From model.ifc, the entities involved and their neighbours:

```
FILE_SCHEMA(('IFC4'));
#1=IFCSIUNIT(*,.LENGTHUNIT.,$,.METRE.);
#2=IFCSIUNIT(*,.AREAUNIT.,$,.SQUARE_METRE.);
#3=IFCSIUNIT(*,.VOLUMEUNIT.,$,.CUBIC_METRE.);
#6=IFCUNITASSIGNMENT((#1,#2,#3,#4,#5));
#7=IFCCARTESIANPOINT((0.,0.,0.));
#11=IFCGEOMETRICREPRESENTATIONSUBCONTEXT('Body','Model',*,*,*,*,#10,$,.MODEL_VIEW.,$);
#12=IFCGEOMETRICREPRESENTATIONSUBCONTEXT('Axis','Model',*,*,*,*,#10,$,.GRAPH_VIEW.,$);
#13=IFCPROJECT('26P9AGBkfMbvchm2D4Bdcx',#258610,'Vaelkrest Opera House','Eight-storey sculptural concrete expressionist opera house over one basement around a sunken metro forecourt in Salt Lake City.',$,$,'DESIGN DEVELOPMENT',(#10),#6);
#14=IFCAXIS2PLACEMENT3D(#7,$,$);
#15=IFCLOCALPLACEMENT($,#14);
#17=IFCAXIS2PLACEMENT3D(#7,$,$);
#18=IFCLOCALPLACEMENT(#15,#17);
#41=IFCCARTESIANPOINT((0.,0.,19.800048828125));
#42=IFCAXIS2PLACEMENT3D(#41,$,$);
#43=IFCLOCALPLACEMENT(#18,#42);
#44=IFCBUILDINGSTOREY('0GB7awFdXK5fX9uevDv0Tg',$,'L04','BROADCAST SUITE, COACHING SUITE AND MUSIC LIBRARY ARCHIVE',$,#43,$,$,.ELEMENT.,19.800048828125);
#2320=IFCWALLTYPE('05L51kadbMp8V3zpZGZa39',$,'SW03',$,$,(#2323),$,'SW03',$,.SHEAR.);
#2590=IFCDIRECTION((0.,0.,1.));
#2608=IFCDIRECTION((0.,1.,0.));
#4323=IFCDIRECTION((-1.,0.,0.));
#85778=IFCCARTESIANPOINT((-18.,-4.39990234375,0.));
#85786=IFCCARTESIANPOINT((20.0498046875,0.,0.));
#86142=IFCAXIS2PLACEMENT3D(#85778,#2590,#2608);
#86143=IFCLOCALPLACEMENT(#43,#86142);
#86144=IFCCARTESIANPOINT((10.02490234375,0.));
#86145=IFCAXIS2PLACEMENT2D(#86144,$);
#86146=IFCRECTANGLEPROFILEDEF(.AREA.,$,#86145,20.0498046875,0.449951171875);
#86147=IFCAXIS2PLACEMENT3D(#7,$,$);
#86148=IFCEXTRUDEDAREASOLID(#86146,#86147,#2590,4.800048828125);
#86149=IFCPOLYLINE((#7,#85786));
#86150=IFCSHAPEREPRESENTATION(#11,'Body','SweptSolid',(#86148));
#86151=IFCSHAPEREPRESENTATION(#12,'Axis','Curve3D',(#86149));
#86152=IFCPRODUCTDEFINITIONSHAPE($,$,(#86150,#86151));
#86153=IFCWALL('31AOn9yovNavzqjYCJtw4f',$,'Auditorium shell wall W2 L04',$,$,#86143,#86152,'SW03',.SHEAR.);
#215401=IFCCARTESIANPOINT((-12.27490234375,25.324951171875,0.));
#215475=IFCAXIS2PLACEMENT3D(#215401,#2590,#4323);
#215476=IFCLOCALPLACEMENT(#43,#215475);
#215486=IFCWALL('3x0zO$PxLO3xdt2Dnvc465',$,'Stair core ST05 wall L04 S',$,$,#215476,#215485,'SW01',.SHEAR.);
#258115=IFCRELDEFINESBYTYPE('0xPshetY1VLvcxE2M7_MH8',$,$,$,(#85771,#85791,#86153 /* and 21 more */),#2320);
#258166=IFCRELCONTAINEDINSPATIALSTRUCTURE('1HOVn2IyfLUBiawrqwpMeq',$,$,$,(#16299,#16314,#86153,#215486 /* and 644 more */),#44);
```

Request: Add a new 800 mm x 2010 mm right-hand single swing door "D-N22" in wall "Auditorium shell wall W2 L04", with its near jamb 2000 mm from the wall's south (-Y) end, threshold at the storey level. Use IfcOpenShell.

```python
import numpy as np
import ifcopenshell
import ifcopenshell.api.feature
import ifcopenshell.api.geometry
import ifcopenshell.api.root
import ifcopenshell.api.spatial
import ifcopenshell.geom
import ifcopenshell.util.element
import ifcopenshell.util.placement
import ifcopenshell.util.representation
import ifcopenshell.util.shape
import ifcopenshell.util.unit

model = ifcopenshell.open("model.ifc")
unit_scale = ifcopenshell.util.unit.calculate_unit_scale(model)
settings = ifcopenshell.geom.settings()


def volume(element):
    """Net volume in cubic metres, openings subtracted."""
    shape = ifcopenshell.geom.create_shape(settings, element)
    return ifcopenshell.util.shape.get_volume(shape.geometry)


wall = model.by_guid("31AOn9yovNavzqjYCJtw4f")
storey = ifcopenshell.util.element.get_container(wall, ifc_class="IfcBuildingStorey")
context = ifcopenshell.util.representation.get_context(model, "Model", "Body", "MODEL_VIEW")
before = volume(wall)

width, height, from_end, sill = 0.8, 2.01, 2, 0.0  # metres

# The wall runs along its own X axis, and the end named is its -X end.
wall_shape = ifcopenshell.geom.create_shape(settings, wall)
x, y, z = ifcopenshell.util.shape.get_vertices(wall_shape.geometry).T
start = x.min() + from_end
face, thickness = float(y.min()), float(y.max() - y.min())
wall_matrix = ifcopenshell.util.placement.get_local_placement(wall.ObjectPlacement)
level = ifcopenshell.util.placement.get_local_placement(storey.ObjectPlacement)[2, 3]


def in_wall(x, y):
    """Placement at x, y metres in the wall's axes, at sill height."""
    matrix = wall_matrix.copy()
    matrix[:, 3] = wall_matrix @ np.array([x / unit_scale, y / unit_scale, 0.0, 1.0])
    matrix[2, 3] = level + sill / unit_scale
    return matrix


# Opening: a box that overshoots both wall faces by 50 mm.
opening = ifcopenshell.api.root.create_entity(model, ifc_class="IfcOpeningElement", predefined_type="OPENING")
box = ifcopenshell.api.geometry.add_wall_representation(
    model, context=context, length=width, height=height, thickness=thickness + 0.1
)
ifcopenshell.api.geometry.assign_representation(model, product=opening, representation=box)
ifcopenshell.api.geometry.edit_object_placement(model, product=opening, matrix=in_wall(start, face - 0.05), is_si=False)
ifcopenshell.api.feature.add_feature(model, feature=opening, element=wall)

door = ifcopenshell.api.root.create_entity(model, ifc_class="IfcDoor", name="D-N22", predefined_type="DOOR")
door.OverallWidth, door.OverallHeight = width / unit_scale, height / unit_scale
door.OperationType = "SINGLE_SWING_RIGHT"
body = ifcopenshell.api.geometry.add_door_representation(
    model,
    context=context,
    overall_width=door.OverallWidth,
    overall_height=door.OverallHeight,
    operation_type="SINGLE_SWING_RIGHT",
    lining_properties={"LiningDepth": thickness / unit_scale, "ThresholdDepth": thickness / unit_scale},
)
ifcopenshell.api.geometry.assign_representation(model, product=door, representation=body)
ifcopenshell.api.spatial.assign_container(model, products=[door], relating_structure=storey)
ifcopenshell.api.feature.add_filling(model, opening=opening, element=door)

# The lining spans the wall, so the door starts at the wall face.
ifcopenshell.api.geometry.edit_object_placement(model, product=door, matrix=in_wall(start, face), is_si=False)

after = volume(wall)

print(f"wall volume {before:.3f} -> {after:.3f} m3")

model.write("model_rev.ifc")
```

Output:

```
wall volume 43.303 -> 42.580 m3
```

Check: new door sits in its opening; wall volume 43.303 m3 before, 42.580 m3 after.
